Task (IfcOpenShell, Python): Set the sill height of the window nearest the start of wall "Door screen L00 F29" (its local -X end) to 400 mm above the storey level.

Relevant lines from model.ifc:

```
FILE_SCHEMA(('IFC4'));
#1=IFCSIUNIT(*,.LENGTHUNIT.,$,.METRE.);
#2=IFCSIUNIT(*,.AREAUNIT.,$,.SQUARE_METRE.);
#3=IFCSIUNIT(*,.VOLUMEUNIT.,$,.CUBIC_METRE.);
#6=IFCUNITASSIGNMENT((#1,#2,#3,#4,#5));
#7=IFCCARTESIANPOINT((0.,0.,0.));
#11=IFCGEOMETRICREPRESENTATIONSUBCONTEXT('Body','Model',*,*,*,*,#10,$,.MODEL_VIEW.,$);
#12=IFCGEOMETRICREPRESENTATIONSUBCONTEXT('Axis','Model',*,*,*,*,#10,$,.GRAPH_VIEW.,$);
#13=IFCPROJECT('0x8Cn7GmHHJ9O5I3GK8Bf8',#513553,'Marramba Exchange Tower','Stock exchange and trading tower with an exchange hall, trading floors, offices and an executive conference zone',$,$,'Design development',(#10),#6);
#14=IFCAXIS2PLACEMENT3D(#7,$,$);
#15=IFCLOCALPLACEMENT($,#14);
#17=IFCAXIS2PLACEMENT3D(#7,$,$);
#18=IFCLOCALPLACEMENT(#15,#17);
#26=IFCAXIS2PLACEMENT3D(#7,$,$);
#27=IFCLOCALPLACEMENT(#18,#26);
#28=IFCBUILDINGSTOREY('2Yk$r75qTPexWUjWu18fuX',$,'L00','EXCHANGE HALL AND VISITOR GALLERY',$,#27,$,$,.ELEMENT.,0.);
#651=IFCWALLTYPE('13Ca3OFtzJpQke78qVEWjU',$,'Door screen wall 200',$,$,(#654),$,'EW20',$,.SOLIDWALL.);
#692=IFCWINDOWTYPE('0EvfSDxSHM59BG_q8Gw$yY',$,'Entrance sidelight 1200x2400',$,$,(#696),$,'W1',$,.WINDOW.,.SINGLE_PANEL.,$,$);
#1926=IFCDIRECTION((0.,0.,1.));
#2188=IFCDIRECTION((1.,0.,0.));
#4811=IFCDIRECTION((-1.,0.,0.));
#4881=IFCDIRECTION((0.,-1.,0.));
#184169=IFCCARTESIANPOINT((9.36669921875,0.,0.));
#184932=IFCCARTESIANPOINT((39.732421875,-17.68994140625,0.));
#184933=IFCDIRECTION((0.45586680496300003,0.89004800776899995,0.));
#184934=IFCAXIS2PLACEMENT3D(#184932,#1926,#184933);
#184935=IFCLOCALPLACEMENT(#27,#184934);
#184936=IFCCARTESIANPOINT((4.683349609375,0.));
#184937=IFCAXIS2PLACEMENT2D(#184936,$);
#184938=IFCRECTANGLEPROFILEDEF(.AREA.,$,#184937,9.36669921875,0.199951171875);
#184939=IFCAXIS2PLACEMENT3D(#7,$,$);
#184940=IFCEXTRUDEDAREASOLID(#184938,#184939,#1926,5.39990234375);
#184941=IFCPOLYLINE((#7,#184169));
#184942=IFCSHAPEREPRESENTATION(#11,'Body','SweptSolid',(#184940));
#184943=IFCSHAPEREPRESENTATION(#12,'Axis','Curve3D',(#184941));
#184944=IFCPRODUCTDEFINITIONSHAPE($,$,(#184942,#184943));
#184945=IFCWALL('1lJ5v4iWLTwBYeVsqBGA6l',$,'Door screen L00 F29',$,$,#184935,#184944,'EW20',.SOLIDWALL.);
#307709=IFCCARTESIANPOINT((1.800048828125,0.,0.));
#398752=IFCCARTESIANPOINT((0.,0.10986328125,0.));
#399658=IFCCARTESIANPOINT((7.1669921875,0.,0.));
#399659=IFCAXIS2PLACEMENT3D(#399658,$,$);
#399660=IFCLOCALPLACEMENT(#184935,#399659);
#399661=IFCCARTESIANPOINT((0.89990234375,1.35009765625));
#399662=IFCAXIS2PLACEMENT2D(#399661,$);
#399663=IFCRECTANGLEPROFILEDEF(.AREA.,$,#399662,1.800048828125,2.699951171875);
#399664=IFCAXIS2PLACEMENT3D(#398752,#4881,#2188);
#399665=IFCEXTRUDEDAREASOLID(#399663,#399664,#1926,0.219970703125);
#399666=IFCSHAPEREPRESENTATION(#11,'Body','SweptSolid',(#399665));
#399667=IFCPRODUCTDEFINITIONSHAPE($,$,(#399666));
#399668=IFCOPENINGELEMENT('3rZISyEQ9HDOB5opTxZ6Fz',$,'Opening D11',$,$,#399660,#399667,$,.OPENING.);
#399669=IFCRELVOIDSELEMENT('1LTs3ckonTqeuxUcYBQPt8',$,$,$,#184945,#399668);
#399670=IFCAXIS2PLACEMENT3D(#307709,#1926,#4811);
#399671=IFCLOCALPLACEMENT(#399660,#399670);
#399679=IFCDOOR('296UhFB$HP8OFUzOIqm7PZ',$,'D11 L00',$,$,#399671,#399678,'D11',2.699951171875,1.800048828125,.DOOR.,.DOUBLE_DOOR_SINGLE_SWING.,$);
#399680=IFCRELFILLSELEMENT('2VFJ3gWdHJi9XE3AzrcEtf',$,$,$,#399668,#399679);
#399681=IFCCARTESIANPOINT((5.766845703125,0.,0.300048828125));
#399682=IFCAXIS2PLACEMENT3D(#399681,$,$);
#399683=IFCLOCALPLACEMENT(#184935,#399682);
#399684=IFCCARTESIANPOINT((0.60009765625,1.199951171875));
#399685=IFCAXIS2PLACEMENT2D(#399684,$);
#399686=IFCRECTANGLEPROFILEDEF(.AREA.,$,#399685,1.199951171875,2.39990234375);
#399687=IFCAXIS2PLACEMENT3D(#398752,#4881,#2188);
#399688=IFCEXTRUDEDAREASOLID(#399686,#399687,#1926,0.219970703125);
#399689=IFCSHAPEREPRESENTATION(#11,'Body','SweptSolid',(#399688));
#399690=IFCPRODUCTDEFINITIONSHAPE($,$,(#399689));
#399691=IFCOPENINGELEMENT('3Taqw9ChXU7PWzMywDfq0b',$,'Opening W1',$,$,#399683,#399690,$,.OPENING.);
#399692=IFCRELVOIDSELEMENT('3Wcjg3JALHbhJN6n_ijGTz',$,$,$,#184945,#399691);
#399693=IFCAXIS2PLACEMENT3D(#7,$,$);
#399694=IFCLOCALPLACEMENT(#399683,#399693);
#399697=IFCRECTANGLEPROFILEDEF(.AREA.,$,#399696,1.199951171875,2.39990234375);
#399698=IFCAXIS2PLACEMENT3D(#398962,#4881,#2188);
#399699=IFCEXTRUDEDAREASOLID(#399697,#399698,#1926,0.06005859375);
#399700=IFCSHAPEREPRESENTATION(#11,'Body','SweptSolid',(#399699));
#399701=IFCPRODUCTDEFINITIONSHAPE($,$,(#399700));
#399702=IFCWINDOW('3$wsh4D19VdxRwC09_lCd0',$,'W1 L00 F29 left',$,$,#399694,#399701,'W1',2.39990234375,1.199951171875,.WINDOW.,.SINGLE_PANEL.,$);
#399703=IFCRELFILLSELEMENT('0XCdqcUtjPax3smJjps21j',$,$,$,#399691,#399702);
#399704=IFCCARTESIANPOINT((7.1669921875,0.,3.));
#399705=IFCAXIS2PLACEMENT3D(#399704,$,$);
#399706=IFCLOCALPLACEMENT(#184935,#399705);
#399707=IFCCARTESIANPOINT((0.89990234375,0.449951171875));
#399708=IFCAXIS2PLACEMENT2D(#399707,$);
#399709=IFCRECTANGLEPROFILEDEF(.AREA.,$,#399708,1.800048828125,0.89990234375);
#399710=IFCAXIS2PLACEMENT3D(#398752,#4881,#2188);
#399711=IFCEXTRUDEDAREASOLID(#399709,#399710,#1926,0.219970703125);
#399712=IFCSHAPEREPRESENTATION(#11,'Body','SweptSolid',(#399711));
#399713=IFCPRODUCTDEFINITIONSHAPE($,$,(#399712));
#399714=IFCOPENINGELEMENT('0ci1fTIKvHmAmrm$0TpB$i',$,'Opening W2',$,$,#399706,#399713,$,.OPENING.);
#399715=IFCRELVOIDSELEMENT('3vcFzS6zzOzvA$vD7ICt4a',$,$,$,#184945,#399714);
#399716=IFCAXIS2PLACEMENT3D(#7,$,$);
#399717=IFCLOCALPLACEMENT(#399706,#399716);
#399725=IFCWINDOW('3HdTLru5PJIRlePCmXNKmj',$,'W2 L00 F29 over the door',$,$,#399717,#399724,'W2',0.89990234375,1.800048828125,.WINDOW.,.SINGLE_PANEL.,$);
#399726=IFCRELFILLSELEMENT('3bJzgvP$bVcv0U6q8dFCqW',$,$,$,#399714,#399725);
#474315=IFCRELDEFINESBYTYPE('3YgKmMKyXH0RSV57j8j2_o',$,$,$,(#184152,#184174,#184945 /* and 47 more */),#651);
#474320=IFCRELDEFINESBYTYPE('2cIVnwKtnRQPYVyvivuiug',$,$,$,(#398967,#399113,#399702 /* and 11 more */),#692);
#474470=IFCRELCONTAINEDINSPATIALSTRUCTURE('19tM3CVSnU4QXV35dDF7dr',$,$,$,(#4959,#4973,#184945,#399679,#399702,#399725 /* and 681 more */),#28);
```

```python
import numpy as np
import ifcopenshell
import ifcopenshell.api.geometry
import ifcopenshell.geom
import ifcopenshell.util.element
import ifcopenshell.util.placement
import ifcopenshell.util.shape
import ifcopenshell.util.unit

model = ifcopenshell.open("model.ifc")
unit_scale = ifcopenshell.util.unit.calculate_unit_scale(model)

window = model.by_id(399702)
opening = window.FillsVoids[0].RelatingOpeningElement
storey = ifcopenshell.util.element.get_container(window, ifc_class="IfcBuildingStorey")
level = ifcopenshell.util.placement.get_local_placement(storey.ObjectPlacement)[2, 3]

# The opening's origin need not be at the sill, so measure its lowest point.
shape = ifcopenshell.geom.create_shape(ifcopenshell.geom.settings(), opening)
bottom = ifcopenshell.util.shape.get_shape_bottom_elevation(shape, shape.geometry) / unit_scale
dz = level + 0.4 / unit_scale - bottom

shift = np.array([0.0, 0.0, dz])
# The window is placed relative to its opening, so it follows when the opening moves.
matrix = ifcopenshell.util.placement.get_local_placement(opening.ObjectPlacement)
matrix[:3, 3] += shift
ifcopenshell.api.geometry.edit_object_placement(
    model, product=opening, matrix=matrix, is_si=False, should_transform_children=True
)

print(f"moved by {dz * unit_scale:+.3f} m")

model.write("model-out.ifc")
```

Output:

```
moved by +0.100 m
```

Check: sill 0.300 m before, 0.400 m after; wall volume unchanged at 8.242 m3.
